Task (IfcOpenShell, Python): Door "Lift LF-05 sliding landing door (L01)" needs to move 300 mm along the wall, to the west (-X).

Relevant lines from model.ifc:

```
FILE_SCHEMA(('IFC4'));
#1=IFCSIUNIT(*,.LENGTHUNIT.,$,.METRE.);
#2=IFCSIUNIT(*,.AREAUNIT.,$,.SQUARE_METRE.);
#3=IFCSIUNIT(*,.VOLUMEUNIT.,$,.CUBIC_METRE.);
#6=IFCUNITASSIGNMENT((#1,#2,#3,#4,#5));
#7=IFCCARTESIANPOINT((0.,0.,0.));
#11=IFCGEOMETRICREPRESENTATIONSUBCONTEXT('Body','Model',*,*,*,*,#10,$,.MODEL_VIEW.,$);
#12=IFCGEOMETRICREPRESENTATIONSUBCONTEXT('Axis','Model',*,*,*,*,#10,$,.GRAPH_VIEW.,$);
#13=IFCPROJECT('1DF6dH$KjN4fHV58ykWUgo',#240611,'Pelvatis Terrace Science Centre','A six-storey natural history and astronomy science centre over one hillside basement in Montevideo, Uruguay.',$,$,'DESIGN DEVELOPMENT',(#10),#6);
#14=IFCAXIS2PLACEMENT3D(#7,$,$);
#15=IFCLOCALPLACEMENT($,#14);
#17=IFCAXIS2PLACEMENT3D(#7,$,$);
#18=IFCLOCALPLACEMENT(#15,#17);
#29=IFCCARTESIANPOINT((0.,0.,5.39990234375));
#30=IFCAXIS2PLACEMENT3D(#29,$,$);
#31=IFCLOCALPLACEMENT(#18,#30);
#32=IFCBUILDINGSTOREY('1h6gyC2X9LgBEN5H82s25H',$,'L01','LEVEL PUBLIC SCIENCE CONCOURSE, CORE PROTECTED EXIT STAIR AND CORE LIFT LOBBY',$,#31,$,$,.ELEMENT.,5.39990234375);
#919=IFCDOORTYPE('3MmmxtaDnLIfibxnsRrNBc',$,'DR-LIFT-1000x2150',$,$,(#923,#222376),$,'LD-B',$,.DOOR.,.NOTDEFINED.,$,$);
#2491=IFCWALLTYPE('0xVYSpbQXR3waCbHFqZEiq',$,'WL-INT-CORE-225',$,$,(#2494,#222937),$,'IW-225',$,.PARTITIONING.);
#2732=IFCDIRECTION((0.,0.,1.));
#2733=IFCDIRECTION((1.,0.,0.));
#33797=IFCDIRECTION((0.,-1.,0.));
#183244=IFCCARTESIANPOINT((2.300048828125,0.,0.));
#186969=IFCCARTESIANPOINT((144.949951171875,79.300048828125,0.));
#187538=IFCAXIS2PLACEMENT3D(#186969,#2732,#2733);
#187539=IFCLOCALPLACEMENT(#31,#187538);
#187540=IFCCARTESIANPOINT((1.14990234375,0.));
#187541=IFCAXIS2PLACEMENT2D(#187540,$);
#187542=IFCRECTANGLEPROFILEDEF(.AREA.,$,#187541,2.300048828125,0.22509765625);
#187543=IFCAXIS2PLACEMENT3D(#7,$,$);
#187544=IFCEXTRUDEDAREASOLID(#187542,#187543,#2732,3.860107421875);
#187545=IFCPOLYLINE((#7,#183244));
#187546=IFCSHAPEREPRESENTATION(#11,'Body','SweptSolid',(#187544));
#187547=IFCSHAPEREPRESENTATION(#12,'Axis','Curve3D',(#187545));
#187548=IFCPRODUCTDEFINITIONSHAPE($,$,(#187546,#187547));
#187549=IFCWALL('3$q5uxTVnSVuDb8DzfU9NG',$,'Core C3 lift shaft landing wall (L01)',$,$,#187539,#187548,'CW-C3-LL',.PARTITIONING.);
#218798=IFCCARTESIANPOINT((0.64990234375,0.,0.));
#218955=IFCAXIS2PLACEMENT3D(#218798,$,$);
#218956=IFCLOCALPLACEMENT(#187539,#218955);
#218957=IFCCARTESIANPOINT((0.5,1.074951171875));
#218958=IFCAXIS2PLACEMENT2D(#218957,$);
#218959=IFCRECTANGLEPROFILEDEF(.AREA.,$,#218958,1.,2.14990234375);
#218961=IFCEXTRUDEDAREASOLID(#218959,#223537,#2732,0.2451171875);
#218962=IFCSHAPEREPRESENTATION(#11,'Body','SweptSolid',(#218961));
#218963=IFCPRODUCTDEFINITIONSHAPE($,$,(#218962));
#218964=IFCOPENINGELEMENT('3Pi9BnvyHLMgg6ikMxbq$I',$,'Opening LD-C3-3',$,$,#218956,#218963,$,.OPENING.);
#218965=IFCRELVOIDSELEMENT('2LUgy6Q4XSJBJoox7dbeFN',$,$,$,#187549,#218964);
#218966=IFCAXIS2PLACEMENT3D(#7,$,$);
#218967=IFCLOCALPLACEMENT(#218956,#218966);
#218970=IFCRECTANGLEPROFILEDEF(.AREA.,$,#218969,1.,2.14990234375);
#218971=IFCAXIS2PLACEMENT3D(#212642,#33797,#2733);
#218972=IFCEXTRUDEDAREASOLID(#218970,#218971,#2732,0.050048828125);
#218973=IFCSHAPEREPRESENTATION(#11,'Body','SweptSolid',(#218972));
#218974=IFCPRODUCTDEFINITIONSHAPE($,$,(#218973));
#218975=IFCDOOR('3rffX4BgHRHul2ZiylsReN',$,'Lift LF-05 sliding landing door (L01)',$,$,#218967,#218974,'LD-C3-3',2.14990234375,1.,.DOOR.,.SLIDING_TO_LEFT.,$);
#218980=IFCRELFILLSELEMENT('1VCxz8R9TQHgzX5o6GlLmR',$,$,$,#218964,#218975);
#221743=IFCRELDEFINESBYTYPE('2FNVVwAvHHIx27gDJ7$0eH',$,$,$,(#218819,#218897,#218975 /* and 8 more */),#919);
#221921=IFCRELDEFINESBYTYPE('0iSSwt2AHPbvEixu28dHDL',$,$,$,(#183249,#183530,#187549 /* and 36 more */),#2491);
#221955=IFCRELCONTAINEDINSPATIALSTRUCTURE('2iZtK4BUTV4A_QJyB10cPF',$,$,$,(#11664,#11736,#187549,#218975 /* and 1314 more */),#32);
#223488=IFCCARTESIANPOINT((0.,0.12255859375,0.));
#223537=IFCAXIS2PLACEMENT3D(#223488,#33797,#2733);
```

```python
import ifcopenshell
import ifcopenshell.api.geometry
import ifcopenshell.util.placement
import ifcopenshell.util.unit

model = ifcopenshell.open("model.ifc")
unit_scale = ifcopenshell.util.unit.calculate_unit_scale(model)

door = model.by_guid("3rffX4BgHRHul2ZiylsReN")
opening = door.FillsVoids[0].RelatingOpeningElement
wall = opening.VoidsElements[0].RelatingBuildingElement

wall_matrix = ifcopenshell.util.placement.get_local_placement(wall.ObjectPlacement)
shift = wall_matrix[:3, 0] * -0.3 / unit_scale
before = ifcopenshell.util.placement.get_local_placement(door.ObjectPlacement)[:3, 3].copy()

# The door is placed relative to its opening, so it follows when the opening moves.
matrix = ifcopenshell.util.placement.get_local_placement(opening.ObjectPlacement)
matrix[:3, 3] += shift
ifcopenshell.api.geometry.edit_object_placement(
    model, product=opening, matrix=matrix, is_si=False, should_transform_children=True
)

after = ifcopenshell.util.placement.get_local_placement(door.ObjectPlacement)[:3, 3]
print("door moved by", (after - before).round(3) + 0.0)

model.write("model_updated.ifc")
```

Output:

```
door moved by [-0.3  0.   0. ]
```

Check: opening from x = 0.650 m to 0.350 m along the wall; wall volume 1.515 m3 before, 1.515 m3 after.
